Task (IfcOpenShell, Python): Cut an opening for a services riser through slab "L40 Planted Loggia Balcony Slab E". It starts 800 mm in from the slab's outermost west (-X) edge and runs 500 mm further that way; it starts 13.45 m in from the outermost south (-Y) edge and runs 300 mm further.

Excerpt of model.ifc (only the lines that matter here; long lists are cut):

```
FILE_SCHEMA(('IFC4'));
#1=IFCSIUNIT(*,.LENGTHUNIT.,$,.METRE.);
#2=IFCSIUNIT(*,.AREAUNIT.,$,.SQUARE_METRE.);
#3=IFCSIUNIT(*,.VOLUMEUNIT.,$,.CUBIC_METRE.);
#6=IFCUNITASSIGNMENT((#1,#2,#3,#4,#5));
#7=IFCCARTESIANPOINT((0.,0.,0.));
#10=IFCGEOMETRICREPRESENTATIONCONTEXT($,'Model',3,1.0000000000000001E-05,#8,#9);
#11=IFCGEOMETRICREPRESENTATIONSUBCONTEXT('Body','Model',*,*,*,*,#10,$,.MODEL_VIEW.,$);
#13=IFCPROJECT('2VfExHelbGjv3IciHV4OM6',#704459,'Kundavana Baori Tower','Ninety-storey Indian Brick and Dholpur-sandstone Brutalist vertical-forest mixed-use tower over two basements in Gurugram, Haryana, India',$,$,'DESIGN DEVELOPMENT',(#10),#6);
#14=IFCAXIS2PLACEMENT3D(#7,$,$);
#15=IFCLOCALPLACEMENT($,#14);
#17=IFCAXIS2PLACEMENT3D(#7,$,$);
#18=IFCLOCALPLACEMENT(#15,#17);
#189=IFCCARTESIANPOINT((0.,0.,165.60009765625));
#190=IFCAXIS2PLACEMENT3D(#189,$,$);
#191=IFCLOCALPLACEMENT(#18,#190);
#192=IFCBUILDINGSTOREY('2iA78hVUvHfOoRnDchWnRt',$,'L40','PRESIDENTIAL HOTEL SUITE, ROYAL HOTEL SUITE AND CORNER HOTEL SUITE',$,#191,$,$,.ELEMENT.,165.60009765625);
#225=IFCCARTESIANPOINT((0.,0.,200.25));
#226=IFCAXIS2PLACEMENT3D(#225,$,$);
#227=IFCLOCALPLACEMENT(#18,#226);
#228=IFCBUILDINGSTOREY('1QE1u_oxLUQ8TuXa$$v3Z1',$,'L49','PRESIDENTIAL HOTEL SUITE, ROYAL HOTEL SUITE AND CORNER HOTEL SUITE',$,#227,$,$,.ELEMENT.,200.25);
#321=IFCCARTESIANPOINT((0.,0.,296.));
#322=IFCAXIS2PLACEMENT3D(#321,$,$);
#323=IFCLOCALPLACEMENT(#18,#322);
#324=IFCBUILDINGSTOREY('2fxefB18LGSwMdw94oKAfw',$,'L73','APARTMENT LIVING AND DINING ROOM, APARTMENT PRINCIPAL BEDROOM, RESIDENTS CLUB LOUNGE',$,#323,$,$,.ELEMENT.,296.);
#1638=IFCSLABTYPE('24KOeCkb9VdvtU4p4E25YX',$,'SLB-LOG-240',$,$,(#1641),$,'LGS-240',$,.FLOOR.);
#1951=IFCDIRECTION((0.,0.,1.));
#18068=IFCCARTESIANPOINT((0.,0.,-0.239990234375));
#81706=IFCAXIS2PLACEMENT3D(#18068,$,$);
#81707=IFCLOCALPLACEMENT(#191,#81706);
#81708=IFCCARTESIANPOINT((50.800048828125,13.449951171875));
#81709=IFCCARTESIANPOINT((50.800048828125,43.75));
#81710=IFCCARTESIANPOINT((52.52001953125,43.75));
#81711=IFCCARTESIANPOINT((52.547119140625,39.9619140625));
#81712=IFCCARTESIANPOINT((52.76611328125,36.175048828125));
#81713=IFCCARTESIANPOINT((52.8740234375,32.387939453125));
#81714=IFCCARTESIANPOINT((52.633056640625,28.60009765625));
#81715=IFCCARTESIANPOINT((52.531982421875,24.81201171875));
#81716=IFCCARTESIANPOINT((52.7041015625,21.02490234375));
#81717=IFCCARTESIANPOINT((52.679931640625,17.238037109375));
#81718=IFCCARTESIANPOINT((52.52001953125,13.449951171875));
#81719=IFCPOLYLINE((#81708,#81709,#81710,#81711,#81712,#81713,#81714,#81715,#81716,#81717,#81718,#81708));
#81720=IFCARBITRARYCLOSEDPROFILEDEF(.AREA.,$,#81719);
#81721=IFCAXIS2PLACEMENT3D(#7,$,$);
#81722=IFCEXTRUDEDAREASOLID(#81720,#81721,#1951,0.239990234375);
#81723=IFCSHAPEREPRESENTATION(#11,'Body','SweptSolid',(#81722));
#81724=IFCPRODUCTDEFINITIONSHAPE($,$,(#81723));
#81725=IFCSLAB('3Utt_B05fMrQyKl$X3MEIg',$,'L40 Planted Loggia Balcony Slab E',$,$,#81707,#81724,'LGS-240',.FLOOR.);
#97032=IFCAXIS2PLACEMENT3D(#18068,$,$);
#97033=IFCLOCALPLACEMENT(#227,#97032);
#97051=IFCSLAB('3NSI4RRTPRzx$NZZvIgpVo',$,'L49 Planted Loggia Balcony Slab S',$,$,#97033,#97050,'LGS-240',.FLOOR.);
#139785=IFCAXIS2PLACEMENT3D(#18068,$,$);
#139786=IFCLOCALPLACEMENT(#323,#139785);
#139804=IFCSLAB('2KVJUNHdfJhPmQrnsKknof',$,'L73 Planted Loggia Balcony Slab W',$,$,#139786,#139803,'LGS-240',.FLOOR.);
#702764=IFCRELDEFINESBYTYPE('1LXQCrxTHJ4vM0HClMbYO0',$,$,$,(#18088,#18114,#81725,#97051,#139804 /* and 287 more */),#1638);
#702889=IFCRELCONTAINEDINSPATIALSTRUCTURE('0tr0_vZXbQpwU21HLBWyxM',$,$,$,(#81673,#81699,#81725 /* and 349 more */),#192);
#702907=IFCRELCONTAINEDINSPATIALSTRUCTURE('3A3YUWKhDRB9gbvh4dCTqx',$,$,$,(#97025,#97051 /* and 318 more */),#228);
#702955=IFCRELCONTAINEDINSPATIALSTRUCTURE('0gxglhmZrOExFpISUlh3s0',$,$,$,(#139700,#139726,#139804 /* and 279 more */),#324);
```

```python
import numpy as np
import ifcopenshell
import ifcopenshell.api.feature
import ifcopenshell.api.geometry
import ifcopenshell.api.root
import ifcopenshell.geom
import ifcopenshell.util.placement
import ifcopenshell.util.representation
import ifcopenshell.util.shape
import ifcopenshell.util.unit

model = ifcopenshell.open("model.ifc")
unit_scale = ifcopenshell.util.unit.calculate_unit_scale(model)
settings = ifcopenshell.geom.settings()


def volume(element):
    """Net volume in cubic metres, openings subtracted."""
    shape = ifcopenshell.geom.create_shape(settings, element)
    return ifcopenshell.util.shape.get_volume(shape.geometry)


slab = model.by_guid("3Utt_B05fMrQyKl$X3MEIg")
before = volume(slab)

# Extent in the slab's own axes, in metres. The edges named are its -X and -Y sides.
slab_shape = ifcopenshell.geom.create_shape(settings, slab)
vertices = ifcopenshell.util.shape.get_vertices(slab_shape.geometry)
x_min, y_min, bottom = vertices.min(axis=0)
top = vertices[:, 2].max()

opening = ifcopenshell.api.root.create_entity(model, ifc_class="IfcOpeningElement", name="Services riser opening", predefined_type="OPENING")
context = ifcopenshell.util.representation.get_context(model, "Model", "Body", "MODEL_VIEW")
width, depth = 0.5, 0.3
outline = [(0.0, 0.0), (width, 0.0), (width, depth), (0.0, depth), (0.0, 0.0)]
# Overshoot both faces by 50 mm so the cut is clean.
shape = ifcopenshell.api.geometry.add_slab_representation(
    model, context=context, depth=top - bottom + 0.1, polyline=outline
)
ifcopenshell.api.geometry.assign_representation(model, product=opening, representation=shape)

matrix = ifcopenshell.util.placement.get_local_placement(slab.ObjectPlacement)
matrix[:, 3] = matrix @ np.append(np.array([x_min + 0.8, y_min + 13.45, bottom - 0.05]) / unit_scale, 1.0)
ifcopenshell.api.geometry.edit_object_placement(model, product=opening, matrix=matrix, is_si=False)
ifcopenshell.api.feature.add_feature(model, feature=opening, element=slab)

after = volume(slab)

print(f"slab volume {before:.3f} -> {after:.3f} m3")

model.write("model_rev.ifc")
```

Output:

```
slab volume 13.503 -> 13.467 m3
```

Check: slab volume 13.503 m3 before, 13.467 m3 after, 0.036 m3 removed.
